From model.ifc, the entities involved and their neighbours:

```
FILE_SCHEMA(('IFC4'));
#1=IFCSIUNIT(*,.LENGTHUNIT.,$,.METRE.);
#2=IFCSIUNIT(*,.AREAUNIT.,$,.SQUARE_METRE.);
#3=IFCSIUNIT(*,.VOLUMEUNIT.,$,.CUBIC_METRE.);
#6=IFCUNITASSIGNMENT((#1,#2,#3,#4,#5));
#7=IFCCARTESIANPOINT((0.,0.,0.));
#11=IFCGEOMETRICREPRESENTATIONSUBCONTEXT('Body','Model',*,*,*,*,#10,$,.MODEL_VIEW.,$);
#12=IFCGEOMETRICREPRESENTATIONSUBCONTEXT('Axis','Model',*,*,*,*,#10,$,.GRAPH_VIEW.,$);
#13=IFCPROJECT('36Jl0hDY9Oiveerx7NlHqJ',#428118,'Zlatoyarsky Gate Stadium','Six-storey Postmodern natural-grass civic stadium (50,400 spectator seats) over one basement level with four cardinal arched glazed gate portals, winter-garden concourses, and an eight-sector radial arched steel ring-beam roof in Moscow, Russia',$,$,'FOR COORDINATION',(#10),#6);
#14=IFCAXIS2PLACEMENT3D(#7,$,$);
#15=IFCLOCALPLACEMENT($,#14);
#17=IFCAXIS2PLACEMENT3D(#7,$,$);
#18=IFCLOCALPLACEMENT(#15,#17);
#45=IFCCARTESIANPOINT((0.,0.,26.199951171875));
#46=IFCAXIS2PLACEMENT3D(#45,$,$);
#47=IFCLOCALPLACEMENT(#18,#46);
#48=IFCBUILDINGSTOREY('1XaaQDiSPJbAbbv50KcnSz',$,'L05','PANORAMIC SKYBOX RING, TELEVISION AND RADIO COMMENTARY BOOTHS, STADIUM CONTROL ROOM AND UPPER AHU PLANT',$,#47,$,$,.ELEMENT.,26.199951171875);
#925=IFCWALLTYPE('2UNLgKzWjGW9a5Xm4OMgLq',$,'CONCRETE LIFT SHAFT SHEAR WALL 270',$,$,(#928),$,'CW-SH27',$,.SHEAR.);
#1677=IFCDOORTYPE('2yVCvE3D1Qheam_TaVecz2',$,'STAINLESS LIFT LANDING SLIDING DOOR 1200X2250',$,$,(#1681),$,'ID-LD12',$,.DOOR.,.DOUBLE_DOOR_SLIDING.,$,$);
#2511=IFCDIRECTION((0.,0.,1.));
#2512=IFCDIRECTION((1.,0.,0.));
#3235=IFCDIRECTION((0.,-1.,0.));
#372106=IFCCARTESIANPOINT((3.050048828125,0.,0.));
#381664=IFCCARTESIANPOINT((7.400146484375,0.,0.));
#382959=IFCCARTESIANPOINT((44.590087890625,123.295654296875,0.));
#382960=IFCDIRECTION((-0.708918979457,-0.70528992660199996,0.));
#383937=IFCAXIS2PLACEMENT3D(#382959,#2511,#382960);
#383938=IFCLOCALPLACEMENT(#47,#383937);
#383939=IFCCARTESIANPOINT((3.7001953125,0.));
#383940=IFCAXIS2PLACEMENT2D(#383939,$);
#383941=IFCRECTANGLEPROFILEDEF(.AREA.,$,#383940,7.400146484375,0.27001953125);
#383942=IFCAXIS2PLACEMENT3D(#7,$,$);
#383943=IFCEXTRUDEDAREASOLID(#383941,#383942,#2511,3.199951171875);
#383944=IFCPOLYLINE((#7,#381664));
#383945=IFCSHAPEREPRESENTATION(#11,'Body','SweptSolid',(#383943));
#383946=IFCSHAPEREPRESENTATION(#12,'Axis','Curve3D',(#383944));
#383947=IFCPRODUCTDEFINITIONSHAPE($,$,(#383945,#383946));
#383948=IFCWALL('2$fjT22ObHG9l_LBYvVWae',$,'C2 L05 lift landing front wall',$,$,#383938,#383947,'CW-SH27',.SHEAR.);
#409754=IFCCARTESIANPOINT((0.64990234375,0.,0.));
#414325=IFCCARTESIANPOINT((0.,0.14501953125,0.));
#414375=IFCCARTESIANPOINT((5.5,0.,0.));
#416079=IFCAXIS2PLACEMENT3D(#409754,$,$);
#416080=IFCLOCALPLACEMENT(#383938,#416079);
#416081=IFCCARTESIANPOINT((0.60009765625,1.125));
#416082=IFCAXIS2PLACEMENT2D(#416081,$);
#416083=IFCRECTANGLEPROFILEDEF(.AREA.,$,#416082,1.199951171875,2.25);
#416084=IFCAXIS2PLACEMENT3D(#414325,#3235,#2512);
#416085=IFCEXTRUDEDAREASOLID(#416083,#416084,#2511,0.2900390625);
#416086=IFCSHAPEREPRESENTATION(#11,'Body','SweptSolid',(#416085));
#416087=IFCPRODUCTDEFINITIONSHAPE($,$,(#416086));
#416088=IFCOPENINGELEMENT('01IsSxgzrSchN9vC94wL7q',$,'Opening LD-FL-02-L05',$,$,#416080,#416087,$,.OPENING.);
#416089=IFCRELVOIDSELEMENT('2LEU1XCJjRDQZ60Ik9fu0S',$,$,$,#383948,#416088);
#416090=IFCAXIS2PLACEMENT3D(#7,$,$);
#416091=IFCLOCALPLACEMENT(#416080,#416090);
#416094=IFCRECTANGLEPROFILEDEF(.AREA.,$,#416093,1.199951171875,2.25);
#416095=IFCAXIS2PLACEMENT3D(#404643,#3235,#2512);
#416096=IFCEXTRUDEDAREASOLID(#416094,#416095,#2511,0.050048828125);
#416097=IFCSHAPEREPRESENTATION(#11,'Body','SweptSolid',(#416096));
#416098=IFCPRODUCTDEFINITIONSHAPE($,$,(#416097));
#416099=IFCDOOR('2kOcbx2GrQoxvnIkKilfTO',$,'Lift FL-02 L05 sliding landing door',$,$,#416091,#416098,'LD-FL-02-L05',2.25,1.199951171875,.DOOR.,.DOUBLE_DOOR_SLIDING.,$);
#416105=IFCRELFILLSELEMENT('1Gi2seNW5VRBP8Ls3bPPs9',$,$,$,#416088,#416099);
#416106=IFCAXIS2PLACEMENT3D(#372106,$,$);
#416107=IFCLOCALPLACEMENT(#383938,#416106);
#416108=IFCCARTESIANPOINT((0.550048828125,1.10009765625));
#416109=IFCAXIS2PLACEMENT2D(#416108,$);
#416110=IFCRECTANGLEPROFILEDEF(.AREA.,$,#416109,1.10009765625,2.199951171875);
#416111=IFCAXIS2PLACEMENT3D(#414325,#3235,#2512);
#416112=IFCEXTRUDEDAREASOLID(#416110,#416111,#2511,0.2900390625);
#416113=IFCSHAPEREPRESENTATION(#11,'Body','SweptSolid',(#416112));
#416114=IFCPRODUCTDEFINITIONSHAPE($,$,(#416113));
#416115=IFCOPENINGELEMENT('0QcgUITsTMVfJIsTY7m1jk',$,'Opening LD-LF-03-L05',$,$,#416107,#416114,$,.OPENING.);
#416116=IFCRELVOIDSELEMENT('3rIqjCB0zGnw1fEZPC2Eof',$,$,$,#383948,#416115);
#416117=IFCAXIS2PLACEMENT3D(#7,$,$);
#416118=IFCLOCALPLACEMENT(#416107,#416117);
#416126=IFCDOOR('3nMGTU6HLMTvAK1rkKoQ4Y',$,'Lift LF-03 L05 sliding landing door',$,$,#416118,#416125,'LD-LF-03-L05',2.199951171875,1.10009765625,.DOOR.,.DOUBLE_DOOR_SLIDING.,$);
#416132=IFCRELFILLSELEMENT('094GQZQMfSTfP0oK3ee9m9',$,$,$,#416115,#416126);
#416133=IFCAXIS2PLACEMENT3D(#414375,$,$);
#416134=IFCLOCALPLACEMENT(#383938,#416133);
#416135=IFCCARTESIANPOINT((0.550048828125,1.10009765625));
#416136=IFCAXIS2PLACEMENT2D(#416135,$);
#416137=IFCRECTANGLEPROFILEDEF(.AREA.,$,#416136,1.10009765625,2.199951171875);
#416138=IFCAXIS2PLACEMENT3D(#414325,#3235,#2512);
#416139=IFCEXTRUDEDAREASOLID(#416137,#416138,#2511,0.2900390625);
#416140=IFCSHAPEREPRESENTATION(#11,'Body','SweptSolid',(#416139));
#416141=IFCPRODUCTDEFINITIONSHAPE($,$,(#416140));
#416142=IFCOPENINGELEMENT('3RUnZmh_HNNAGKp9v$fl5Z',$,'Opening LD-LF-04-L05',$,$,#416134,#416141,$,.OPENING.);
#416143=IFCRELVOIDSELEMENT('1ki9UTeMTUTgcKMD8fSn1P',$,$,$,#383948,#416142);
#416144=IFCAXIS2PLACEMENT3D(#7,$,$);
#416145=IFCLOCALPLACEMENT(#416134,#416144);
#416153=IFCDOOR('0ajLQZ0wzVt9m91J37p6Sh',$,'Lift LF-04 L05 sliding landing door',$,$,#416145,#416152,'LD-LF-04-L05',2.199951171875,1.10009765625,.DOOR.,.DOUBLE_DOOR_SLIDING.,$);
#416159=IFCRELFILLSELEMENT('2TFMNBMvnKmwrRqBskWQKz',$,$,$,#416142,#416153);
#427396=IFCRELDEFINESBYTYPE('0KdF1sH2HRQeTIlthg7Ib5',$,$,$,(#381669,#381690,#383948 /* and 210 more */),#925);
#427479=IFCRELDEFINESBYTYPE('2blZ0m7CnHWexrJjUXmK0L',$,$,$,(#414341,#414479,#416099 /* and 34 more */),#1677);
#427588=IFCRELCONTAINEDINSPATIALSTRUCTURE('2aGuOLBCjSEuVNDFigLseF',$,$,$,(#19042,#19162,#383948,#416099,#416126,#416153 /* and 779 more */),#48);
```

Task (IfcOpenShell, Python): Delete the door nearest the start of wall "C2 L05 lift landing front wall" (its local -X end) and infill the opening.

```python
import ifcopenshell
import ifcopenshell.api.feature
import ifcopenshell.api.root
import ifcopenshell.geom
import ifcopenshell.util.shape

model = ifcopenshell.open("model.ifc")
settings = ifcopenshell.geom.settings()


def volume(element):
    """Net volume in cubic metres, openings subtracted."""
    shape = ifcopenshell.geom.create_shape(settings, element)
    return ifcopenshell.util.shape.get_volume(shape.geometry)


door = model.by_guid("2kOcbx2GrQoxvnIkKilfTO")
opening = door.FillsVoids[0].RelatingOpeningElement
wall = opening.VoidsElements[0].RelatingBuildingElement
before = volume(wall)

ifcopenshell.api.root.remove_product(model, product=door)
ifcopenshell.api.feature.remove_feature(model, feature=opening)

after = volume(wall)

print(f"wall volume {before:.3f} -> {after:.3f} m3")

model.write("model_edited.ifc")
```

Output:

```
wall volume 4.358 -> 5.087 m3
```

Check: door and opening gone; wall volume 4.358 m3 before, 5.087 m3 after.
